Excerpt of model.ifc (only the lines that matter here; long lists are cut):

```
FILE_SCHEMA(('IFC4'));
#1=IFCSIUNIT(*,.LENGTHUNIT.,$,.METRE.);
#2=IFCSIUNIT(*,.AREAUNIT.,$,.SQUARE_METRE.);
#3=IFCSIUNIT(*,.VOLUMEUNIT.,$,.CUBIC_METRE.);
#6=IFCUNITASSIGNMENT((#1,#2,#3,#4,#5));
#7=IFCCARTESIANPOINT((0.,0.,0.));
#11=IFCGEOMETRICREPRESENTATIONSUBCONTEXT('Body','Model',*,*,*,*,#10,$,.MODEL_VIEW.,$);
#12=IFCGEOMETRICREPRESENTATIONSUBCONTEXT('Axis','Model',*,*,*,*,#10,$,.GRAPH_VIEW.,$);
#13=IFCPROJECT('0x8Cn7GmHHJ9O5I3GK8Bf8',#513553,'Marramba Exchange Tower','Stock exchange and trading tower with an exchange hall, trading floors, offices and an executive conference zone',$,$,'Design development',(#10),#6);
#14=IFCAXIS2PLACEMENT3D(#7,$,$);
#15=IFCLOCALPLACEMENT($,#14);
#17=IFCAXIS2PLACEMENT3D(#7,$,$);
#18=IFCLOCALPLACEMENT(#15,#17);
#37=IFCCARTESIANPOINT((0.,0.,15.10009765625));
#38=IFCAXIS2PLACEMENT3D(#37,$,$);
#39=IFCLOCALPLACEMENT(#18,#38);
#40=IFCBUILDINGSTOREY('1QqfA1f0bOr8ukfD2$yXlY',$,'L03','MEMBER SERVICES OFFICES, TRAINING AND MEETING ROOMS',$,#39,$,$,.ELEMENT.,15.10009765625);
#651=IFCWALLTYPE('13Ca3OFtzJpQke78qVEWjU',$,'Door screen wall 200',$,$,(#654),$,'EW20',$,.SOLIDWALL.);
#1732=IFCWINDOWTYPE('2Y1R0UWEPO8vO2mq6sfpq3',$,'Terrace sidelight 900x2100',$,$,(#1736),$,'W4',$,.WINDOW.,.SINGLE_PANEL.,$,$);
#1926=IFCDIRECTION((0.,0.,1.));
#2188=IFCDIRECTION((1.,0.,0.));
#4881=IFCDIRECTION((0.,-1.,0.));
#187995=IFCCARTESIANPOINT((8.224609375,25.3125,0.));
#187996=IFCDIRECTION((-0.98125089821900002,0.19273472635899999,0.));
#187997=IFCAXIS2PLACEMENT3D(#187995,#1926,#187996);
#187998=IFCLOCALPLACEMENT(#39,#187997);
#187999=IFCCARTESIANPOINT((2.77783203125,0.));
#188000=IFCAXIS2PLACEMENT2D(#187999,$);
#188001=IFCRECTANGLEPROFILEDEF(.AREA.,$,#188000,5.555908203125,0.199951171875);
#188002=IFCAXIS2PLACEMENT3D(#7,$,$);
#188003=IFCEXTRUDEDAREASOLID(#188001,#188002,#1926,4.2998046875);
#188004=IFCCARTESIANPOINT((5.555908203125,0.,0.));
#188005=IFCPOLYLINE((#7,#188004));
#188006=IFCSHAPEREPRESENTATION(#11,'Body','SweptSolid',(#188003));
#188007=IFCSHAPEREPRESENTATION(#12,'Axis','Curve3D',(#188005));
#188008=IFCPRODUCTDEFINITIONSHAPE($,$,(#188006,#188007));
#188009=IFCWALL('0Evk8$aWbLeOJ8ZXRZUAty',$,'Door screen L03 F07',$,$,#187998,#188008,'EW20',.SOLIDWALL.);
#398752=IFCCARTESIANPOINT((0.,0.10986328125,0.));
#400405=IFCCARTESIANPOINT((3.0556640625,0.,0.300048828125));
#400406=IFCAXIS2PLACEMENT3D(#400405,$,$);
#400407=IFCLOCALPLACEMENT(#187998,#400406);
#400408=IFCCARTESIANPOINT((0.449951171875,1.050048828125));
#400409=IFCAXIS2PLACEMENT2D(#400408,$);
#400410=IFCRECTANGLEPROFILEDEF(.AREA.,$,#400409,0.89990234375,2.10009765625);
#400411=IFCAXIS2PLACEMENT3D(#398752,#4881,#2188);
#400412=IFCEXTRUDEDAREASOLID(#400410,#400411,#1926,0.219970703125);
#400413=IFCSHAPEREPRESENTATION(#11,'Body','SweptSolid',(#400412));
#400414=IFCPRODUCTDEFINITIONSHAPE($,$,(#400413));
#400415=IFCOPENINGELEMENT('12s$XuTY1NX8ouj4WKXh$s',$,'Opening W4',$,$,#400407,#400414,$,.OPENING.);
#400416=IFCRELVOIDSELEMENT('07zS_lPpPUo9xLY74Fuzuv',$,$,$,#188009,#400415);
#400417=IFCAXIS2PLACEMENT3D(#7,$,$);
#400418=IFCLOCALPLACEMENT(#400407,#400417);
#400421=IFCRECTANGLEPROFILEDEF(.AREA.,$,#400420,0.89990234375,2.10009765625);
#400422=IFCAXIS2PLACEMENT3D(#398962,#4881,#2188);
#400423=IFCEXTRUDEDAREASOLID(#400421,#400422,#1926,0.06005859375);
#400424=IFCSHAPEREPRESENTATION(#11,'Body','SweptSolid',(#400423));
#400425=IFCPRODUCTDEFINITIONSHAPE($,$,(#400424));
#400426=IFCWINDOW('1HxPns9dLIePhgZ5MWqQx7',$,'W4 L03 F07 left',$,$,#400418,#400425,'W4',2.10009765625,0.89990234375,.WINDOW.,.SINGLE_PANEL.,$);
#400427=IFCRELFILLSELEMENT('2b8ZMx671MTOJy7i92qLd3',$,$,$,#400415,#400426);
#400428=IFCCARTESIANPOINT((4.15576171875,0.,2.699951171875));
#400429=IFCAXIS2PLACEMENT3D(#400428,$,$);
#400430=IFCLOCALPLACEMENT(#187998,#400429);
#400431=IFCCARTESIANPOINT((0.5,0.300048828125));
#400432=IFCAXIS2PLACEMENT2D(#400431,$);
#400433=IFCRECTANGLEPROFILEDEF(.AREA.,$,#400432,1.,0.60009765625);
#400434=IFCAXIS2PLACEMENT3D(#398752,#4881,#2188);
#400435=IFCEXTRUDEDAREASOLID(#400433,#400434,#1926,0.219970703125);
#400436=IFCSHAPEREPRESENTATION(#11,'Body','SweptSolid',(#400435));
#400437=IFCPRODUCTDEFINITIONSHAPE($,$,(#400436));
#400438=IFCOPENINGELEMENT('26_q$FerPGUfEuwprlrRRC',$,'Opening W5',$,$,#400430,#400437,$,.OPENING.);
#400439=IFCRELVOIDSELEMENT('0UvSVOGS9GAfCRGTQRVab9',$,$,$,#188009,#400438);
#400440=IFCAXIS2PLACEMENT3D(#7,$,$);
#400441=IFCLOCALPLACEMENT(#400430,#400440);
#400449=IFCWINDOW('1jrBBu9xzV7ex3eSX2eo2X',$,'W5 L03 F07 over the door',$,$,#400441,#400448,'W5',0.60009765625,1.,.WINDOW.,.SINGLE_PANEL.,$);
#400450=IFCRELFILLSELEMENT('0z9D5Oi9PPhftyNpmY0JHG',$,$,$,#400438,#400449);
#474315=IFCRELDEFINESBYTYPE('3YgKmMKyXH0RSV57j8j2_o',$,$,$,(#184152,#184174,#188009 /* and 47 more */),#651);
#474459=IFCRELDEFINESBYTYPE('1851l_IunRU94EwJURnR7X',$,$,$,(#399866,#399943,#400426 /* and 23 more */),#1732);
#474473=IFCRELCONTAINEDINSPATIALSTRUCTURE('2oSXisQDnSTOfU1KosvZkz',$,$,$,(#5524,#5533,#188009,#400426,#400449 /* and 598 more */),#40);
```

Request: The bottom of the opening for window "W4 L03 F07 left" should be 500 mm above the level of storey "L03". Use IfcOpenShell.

```python
import numpy as np
import ifcopenshell
import ifcopenshell.api.geometry
import ifcopenshell.geom
import ifcopenshell.util.element
import ifcopenshell.util.placement
import ifcopenshell.util.shape
import ifcopenshell.util.unit

model = ifcopenshell.open("model.ifc")
unit_scale = ifcopenshell.util.unit.calculate_unit_scale(model)

window = model.by_guid("1HxPns9dLIePhgZ5MWqQx7")
opening = window.FillsVoids[0].RelatingOpeningElement
storey = ifcopenshell.util.element.get_container(window, ifc_class="IfcBuildingStorey")
level = ifcopenshell.util.placement.get_local_placement(storey.ObjectPlacement)[2, 3]

# The opening's origin need not be at the sill, so measure its lowest point.
shape = ifcopenshell.geom.create_shape(ifcopenshell.geom.settings(), opening)
bottom = ifcopenshell.util.shape.get_shape_bottom_elevation(shape, shape.geometry) / unit_scale
dz = level + 0.5 / unit_scale - bottom

shift = np.array([0.0, 0.0, dz])
# The window is placed relative to its opening, so it follows when the opening moves.
matrix = ifcopenshell.util.placement.get_local_placement(opening.ObjectPlacement)
matrix[:3, 3] += shift
ifcopenshell.api.geometry.edit_object_placement(
    model, product=opening, matrix=matrix, is_si=False, should_transform_children=True
)

print(f"moved by {dz * unit_scale:+.3f} m")

model.write("model-out.ifc")
```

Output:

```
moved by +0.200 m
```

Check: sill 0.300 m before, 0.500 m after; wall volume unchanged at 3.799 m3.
